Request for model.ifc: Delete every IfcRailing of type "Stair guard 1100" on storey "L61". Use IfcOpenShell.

First a look at what the model holds.

```python
import ifcopenshell
import ifcopenshell.util.element

model = ifcopenshell.open("model.ifc")
print(model.schema)
storey = next(s for s in model.by_type("IfcBuildingStorey") if s.Name == "L61")
railings = [e for e in ifcopenshell.util.element.get_decomposition(storey) if e.is_a("IfcRailing")]
seen = {}
for e in railings:
    element_type = ifcopenshell.util.element.get_type(e)
    name = element_type.Name if element_type not in (None, e) else None
    seen[name] = seen.get(name, 0) + 1
for name, count in sorted(seen.items(), key=str):
    print(count, "x", name)
```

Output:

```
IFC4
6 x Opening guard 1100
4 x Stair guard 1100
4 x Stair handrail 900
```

```python
import ifcopenshell
import ifcopenshell.api.root
import ifcopenshell.util.element

model = ifcopenshell.open("model.ifc")

storey = next(s for s in model.by_type("IfcBuildingStorey") if s.Name == "L61")
railings = [e for e in ifcopenshell.util.element.get_decomposition(storey) if e.is_a("IfcRailing")]
targets = [e for e in railings if (t := ifcopenshell.util.element.get_type(e)) not in (None, e) and t.Name == "Stair guard 1100"]

for e in targets:
    ifcopenshell.api.root.remove_product(model, product=e)
print(len(targets), "removed")

model.write("model_edited.ifc")
```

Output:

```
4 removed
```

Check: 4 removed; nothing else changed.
